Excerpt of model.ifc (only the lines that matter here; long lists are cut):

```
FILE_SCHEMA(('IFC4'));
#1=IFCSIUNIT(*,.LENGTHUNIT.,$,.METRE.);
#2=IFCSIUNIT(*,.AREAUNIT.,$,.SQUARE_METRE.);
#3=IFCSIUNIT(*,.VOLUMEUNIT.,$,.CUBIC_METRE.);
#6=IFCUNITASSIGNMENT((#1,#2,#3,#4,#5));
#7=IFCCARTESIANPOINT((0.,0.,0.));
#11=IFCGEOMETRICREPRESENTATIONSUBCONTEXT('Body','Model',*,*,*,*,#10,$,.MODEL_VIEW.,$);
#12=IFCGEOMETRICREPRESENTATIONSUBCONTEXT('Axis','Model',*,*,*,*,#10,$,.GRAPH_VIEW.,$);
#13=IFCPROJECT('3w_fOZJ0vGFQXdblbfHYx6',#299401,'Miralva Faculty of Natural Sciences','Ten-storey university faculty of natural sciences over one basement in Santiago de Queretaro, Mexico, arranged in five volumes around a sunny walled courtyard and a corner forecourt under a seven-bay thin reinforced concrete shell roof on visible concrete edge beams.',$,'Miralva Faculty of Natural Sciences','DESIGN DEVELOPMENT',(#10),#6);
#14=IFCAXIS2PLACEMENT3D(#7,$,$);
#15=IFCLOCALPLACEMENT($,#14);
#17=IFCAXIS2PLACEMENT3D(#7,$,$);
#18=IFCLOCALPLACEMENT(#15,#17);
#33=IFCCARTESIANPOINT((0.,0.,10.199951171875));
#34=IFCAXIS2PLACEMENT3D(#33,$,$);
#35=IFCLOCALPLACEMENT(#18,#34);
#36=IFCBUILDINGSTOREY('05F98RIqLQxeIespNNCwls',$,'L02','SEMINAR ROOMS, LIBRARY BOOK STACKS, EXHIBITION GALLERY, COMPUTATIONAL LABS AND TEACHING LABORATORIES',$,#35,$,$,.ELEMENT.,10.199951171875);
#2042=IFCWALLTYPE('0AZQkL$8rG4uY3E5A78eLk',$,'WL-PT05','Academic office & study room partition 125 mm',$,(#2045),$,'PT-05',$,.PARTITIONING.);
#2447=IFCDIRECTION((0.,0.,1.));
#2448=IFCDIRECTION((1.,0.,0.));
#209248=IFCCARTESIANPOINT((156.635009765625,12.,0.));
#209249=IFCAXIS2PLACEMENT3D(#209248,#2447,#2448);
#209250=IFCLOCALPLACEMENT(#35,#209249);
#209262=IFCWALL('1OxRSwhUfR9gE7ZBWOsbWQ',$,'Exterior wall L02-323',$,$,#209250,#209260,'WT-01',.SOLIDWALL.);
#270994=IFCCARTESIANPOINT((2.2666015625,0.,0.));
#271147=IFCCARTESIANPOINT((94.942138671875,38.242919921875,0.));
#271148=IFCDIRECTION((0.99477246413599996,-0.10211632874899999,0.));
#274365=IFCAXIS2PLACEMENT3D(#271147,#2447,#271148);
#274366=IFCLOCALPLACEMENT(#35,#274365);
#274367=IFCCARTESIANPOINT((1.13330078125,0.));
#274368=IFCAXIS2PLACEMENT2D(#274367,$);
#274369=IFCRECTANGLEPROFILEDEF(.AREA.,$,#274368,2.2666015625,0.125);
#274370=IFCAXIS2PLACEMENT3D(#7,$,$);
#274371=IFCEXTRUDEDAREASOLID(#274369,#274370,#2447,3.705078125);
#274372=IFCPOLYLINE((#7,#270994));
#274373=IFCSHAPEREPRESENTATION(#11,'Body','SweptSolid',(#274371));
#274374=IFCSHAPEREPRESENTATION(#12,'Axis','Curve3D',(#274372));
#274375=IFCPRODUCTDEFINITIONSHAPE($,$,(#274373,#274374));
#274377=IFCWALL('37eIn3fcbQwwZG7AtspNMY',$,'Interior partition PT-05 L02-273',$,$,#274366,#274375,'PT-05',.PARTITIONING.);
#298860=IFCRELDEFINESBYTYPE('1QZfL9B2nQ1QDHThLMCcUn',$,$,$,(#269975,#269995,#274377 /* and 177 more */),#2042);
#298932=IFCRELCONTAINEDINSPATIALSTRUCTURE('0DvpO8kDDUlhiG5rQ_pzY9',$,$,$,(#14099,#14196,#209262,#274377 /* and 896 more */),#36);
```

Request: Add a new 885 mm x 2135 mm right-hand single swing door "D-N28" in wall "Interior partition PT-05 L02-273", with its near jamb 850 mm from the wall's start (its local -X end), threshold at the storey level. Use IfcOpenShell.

```python
import numpy as np
import ifcopenshell
import ifcopenshell.api.feature
import ifcopenshell.api.geometry
import ifcopenshell.api.root
import ifcopenshell.api.spatial
import ifcopenshell.geom
import ifcopenshell.util.element
import ifcopenshell.util.placement
import ifcopenshell.util.representation
import ifcopenshell.util.shape
import ifcopenshell.util.unit

model = ifcopenshell.open("model.ifc")
unit_scale = ifcopenshell.util.unit.calculate_unit_scale(model)
settings = ifcopenshell.geom.settings()


def volume(element):
    """Net volume in cubic metres, openings subtracted."""
    shape = ifcopenshell.geom.create_shape(settings, element)
    return ifcopenshell.util.shape.get_volume(shape.geometry)


wall = model.by_id(274377)
storey = ifcopenshell.util.element.get_container(wall, ifc_class="IfcBuildingStorey")
context = ifcopenshell.util.representation.get_context(model, "Model", "Body", "MODEL_VIEW")
before = volume(wall)

width, height, from_end, sill = 0.885, 2.135, 0.85, 0.0  # metres

# The wall runs along its own X axis, and the end named is its -X end.
wall_shape = ifcopenshell.geom.create_shape(settings, wall)
x, y, z = ifcopenshell.util.shape.get_vertices(wall_shape.geometry).T
start = x.min() + from_end
face, thickness = float(y.min()), float(y.max() - y.min())
wall_matrix = ifcopenshell.util.placement.get_local_placement(wall.ObjectPlacement)
level = ifcopenshell.util.placement.get_local_placement(storey.ObjectPlacement)[2, 3]


def in_wall(x, y):
    """Placement at x, y metres in the wall's axes, at sill height."""
    matrix = wall_matrix.copy()
    matrix[:, 3] = wall_matrix @ np.array([x / unit_scale, y / unit_scale, 0.0, 1.0])
    matrix[2, 3] = level + sill / unit_scale
    return matrix


# Opening: a box that overshoots both wall faces by 50 mm.
opening = ifcopenshell.api.root.create_entity(model, ifc_class="IfcOpeningElement", predefined_type="OPENING")
box = ifcopenshell.api.geometry.add_wall_representation(
    model, context=context, length=width, height=height, thickness=thickness + 0.1
)
ifcopenshell.api.geometry.assign_representation(model, product=opening, representation=box)
ifcopenshell.api.geometry.edit_object_placement(model, product=opening, matrix=in_wall(start, face - 0.05), is_si=False)
ifcopenshell.api.feature.add_feature(model, feature=opening, element=wall)

door = ifcopenshell.api.root.create_entity(model, ifc_class="IfcDoor", name="D-N28", predefined_type="DOOR")
door.OverallWidth, door.OverallHeight = width / unit_scale, height / unit_scale
door.OperationType = "SINGLE_SWING_RIGHT"
body = ifcopenshell.api.geometry.add_door_representation(
    model,
    context=context,
    overall_width=door.OverallWidth,
    overall_height=door.OverallHeight,
    operation_type="SINGLE_SWING_RIGHT",
    lining_properties={"LiningDepth": thickness / unit_scale, "ThresholdDepth": thickness / unit_scale},
)
ifcopenshell.api.geometry.assign_representation(model, product=door, representation=body)
ifcopenshell.api.spatial.assign_container(model, products=[door], relating_structure=storey)
ifcopenshell.api.feature.add_filling(model, opening=opening, element=door)

# The lining spans the wall, so the door starts at the wall face.
ifcopenshell.api.geometry.edit_object_placement(model, product=door, matrix=in_wall(start, face), is_si=False)

after = volume(wall)

print(f"wall volume {before:.3f} -> {after:.3f} m3")

model.write("model_rev.ifc")
```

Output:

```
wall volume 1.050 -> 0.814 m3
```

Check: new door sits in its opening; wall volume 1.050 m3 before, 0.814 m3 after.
